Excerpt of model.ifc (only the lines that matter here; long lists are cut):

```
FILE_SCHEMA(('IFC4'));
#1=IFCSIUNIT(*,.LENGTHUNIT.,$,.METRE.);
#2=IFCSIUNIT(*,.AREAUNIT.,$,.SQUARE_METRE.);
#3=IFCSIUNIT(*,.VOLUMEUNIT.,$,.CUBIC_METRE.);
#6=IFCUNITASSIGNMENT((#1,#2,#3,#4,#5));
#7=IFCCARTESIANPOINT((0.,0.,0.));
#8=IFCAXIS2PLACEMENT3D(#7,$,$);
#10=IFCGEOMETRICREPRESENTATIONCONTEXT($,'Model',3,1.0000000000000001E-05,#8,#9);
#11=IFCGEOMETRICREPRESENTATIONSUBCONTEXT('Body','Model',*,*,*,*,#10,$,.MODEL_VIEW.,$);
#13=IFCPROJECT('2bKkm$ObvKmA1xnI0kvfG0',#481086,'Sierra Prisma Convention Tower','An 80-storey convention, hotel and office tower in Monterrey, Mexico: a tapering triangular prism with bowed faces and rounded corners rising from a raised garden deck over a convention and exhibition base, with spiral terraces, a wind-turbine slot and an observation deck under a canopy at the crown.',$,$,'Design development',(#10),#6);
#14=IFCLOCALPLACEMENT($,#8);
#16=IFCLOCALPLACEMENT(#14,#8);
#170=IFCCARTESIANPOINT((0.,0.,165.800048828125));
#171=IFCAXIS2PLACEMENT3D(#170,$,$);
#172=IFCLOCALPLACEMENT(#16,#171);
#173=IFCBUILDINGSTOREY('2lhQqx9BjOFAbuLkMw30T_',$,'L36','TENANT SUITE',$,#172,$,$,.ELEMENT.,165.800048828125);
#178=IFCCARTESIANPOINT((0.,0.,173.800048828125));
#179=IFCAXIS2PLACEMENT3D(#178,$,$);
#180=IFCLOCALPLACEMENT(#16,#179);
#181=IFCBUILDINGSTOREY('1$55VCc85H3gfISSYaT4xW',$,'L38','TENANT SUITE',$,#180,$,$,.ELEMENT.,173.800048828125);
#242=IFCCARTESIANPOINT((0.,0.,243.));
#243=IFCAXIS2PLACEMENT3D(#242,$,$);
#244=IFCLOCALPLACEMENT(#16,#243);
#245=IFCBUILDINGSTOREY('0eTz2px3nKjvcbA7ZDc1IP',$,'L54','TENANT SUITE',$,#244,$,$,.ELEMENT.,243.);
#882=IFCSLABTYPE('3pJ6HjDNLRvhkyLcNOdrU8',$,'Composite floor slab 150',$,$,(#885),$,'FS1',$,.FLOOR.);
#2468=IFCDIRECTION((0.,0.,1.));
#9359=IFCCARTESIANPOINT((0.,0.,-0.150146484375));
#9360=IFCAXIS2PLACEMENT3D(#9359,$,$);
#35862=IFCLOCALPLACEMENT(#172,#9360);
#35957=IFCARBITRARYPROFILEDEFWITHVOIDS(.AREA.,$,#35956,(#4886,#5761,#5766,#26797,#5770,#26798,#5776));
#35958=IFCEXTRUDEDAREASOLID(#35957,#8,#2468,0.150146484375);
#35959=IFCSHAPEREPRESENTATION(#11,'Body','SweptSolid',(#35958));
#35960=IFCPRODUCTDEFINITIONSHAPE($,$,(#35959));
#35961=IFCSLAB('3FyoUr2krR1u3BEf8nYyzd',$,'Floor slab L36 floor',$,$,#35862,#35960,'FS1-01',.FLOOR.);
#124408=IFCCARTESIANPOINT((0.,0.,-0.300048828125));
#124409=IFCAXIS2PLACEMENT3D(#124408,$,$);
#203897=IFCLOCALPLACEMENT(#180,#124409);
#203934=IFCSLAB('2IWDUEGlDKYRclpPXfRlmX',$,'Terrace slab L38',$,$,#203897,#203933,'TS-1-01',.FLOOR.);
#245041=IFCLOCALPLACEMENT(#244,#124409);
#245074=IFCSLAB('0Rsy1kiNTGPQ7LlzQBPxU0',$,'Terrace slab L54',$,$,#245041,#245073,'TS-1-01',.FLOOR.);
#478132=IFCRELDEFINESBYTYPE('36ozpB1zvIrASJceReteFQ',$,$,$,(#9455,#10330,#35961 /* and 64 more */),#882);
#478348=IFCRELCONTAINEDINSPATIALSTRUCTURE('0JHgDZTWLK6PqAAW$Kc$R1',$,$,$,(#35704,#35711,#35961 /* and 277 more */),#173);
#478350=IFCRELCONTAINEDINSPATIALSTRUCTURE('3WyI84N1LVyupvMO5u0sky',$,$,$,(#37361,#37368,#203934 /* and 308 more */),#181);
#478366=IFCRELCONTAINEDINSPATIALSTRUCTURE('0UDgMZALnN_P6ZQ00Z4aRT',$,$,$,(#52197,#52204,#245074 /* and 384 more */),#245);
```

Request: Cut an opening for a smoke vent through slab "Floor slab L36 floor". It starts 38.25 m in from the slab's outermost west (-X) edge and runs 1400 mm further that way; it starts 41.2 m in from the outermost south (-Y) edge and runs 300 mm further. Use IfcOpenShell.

```python
import numpy as np
import ifcopenshell
import ifcopenshell.api.feature
import ifcopenshell.api.geometry
import ifcopenshell.api.root
import ifcopenshell.geom
import ifcopenshell.util.placement
import ifcopenshell.util.representation
import ifcopenshell.util.shape
import ifcopenshell.util.unit

model = ifcopenshell.open("model.ifc")
unit_scale = ifcopenshell.util.unit.calculate_unit_scale(model)
settings = ifcopenshell.geom.settings()


def volume(element):
    """Net volume in cubic metres, openings subtracted."""
    shape = ifcopenshell.geom.create_shape(settings, element)
    return ifcopenshell.util.shape.get_volume(shape.geometry)


slab = model.by_guid("3FyoUr2krR1u3BEf8nYyzd")
before = volume(slab)

# Extent in the slab's own axes, in metres. The edges named are its -X and -Y sides.
slab_shape = ifcopenshell.geom.create_shape(settings, slab)
vertices = ifcopenshell.util.shape.get_vertices(slab_shape.geometry)
x_min, y_min, bottom = vertices.min(axis=0)
top = vertices[:, 2].max()

opening = ifcopenshell.api.root.create_entity(model, ifc_class="IfcOpeningElement", name="Smoke vent opening", predefined_type="OPENING")
context = ifcopenshell.util.representation.get_context(model, "Model", "Body", "MODEL_VIEW")
width, depth = 1.4, 0.3
outline = [(0.0, 0.0), (width, 0.0), (width, depth), (0.0, depth), (0.0, 0.0)]
# Overshoot both faces by 50 mm so the cut is clean.
shape = ifcopenshell.api.geometry.add_slab_representation(
    model, context=context, depth=top - bottom + 0.1, polyline=outline
)
ifcopenshell.api.geometry.assign_representation(model, product=opening, representation=shape)

matrix = ifcopenshell.util.placement.get_local_placement(slab.ObjectPlacement)
matrix[:, 3] = matrix @ np.append(np.array([x_min + 38.25, y_min + 41.2, bottom - 0.05]) / unit_scale, 1.0)
ifcopenshell.api.geometry.edit_object_placement(model, product=opening, matrix=matrix, is_si=False)
ifcopenshell.api.feature.add_feature(model, feature=opening, element=slab)

after = volume(slab)

print(f"slab volume {before:.3f} -> {after:.3f} m3")

model.write("model_updated.ifc")
```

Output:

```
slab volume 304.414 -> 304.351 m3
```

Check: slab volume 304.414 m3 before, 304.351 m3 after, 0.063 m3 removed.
